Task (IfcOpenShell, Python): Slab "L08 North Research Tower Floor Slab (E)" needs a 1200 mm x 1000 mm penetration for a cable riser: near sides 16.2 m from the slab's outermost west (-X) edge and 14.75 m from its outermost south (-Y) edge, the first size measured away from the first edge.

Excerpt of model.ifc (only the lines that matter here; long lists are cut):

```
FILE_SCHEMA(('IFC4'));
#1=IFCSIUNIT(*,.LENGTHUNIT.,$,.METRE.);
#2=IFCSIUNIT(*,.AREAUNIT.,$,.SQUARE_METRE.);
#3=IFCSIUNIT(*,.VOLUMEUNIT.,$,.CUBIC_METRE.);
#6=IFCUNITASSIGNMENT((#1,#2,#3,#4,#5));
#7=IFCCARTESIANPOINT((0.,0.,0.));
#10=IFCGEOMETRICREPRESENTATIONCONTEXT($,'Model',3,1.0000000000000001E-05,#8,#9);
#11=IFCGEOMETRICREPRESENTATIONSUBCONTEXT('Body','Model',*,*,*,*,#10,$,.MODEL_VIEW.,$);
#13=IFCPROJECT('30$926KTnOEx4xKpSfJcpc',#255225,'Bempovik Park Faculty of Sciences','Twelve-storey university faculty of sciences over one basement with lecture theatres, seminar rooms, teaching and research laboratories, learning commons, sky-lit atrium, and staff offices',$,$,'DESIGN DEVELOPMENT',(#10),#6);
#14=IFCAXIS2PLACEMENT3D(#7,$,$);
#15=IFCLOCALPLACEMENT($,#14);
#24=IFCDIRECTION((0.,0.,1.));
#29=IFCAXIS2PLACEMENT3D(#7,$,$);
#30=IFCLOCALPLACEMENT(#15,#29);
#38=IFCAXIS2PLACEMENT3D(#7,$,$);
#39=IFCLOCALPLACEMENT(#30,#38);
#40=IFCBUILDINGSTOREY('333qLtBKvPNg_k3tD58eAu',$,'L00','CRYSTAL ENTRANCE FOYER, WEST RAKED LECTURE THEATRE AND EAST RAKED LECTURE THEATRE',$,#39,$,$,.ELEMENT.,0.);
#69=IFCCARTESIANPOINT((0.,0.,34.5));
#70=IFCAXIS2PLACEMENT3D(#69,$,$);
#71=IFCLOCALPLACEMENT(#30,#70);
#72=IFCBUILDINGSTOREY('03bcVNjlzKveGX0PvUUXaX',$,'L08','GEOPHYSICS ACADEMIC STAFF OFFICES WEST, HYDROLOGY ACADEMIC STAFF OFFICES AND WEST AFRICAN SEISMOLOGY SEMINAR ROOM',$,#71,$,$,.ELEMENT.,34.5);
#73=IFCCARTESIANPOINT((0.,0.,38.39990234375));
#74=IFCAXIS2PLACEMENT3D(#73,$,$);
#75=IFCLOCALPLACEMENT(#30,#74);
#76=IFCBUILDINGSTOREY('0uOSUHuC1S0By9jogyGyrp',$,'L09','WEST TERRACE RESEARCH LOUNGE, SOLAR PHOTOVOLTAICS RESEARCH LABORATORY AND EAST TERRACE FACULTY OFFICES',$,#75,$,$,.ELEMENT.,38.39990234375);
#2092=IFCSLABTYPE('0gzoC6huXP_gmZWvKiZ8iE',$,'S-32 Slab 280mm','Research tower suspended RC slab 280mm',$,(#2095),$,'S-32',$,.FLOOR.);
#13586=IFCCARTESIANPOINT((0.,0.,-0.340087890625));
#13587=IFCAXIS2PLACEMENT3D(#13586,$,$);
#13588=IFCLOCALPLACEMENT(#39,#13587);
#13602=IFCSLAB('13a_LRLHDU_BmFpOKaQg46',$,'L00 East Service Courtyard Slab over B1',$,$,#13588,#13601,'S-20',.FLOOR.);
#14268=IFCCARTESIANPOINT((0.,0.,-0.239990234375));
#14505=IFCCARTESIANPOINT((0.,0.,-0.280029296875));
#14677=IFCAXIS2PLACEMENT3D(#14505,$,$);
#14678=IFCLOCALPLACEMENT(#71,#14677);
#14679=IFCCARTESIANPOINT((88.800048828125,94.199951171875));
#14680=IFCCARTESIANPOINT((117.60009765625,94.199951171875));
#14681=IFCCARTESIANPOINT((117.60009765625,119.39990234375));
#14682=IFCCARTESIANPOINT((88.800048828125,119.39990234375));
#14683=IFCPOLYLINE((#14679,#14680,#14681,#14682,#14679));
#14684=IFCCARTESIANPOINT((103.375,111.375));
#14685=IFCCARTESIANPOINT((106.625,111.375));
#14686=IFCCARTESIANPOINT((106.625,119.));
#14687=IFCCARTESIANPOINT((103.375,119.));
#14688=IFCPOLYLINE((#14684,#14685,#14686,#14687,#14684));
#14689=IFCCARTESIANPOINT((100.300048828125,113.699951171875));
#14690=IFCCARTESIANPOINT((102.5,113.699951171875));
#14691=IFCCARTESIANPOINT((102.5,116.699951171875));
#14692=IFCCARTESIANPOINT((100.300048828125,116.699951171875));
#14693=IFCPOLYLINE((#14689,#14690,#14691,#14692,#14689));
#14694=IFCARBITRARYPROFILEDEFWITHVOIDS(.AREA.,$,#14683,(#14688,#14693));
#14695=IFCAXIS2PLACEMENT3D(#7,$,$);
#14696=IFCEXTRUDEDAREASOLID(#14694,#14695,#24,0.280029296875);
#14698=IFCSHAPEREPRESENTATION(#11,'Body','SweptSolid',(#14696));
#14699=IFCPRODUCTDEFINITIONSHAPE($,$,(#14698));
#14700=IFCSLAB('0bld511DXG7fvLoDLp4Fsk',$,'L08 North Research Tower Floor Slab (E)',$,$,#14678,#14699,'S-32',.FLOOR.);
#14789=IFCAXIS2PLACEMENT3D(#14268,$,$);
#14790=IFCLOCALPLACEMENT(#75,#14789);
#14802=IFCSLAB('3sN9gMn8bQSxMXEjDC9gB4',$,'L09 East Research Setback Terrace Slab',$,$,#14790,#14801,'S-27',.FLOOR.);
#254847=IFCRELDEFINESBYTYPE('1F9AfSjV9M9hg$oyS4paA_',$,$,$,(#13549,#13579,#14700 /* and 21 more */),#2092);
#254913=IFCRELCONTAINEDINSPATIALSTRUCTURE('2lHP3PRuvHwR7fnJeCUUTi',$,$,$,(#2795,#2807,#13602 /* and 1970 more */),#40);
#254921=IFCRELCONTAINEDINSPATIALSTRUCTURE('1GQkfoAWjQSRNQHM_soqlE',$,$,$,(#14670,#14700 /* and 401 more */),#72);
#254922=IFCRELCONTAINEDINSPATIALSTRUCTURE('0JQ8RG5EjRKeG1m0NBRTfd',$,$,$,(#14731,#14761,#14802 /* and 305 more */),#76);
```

```python
import numpy as np
import ifcopenshell
import ifcopenshell.api.feature
import ifcopenshell.api.geometry
import ifcopenshell.api.root
import ifcopenshell.geom
import ifcopenshell.util.placement
import ifcopenshell.util.representation
import ifcopenshell.util.shape
import ifcopenshell.util.unit

model = ifcopenshell.open("model.ifc")
unit_scale = ifcopenshell.util.unit.calculate_unit_scale(model)
settings = ifcopenshell.geom.settings()


def volume(element):
    """Net volume in cubic metres, openings subtracted."""
    shape = ifcopenshell.geom.create_shape(settings, element)
    return ifcopenshell.util.shape.get_volume(shape.geometry)


slab = model.by_guid("0bld511DXG7fvLoDLp4Fsk")
before = volume(slab)

# Extent in the slab's own axes, in metres. The edges named are its -X and -Y sides.
slab_shape = ifcopenshell.geom.create_shape(settings, slab)
vertices = ifcopenshell.util.shape.get_vertices(slab_shape.geometry)
x_min, y_min, bottom = vertices.min(axis=0)
top = vertices[:, 2].max()

opening = ifcopenshell.api.root.create_entity(model, ifc_class="IfcOpeningElement", name="Cable riser opening", predefined_type="OPENING")
context = ifcopenshell.util.representation.get_context(model, "Model", "Body", "MODEL_VIEW")
width, depth = 1.2, 1
outline = [(0.0, 0.0), (width, 0.0), (width, depth), (0.0, depth), (0.0, 0.0)]
# Overshoot both faces by 50 mm so the cut is clean.
shape = ifcopenshell.api.geometry.add_slab_representation(
    model, context=context, depth=top - bottom + 0.1, polyline=outline
)
ifcopenshell.api.geometry.assign_representation(model, product=opening, representation=shape)

matrix = ifcopenshell.util.placement.get_local_placement(slab.ObjectPlacement)
matrix[:, 3] = matrix @ np.append(np.array([x_min + 16.2, y_min + 14.75, bottom - 0.05]) / unit_scale, 1.0)
ifcopenshell.api.geometry.edit_object_placement(model, product=opening, matrix=matrix, is_si=False)
ifcopenshell.api.feature.add_feature(model, feature=opening, element=slab)

after = volume(slab)

print(f"slab volume {before:.3f} -> {after:.3f} m3")

model.write("model_rev.ifc")
```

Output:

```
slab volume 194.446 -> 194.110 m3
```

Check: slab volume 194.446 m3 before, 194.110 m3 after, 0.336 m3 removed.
